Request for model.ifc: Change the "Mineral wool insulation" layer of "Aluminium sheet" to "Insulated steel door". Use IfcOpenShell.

First a look at what the model holds.

```python
import ifcopenshell
import ifcopenshell.util.element

model = ifcopenshell.open("model.ifc")
print(model.schema)
for layer_set in model.by_type("IfcMaterialLayerSet"):
    if layer_set.LayerSetName == "Aluminium sheet":
        for layer in layer_set.MaterialLayers:
            print(layer.id(), layer.Material and layer.Material.Name, layer.LayerThickness, sep=" | ")
        print(len(ifcopenshell.util.element.get_elements_by_material(model, layer_set)), "elements and types use it")
print(sorted(m.Name for m in model.by_type("IfcMaterial") if m.Name)[:60])
```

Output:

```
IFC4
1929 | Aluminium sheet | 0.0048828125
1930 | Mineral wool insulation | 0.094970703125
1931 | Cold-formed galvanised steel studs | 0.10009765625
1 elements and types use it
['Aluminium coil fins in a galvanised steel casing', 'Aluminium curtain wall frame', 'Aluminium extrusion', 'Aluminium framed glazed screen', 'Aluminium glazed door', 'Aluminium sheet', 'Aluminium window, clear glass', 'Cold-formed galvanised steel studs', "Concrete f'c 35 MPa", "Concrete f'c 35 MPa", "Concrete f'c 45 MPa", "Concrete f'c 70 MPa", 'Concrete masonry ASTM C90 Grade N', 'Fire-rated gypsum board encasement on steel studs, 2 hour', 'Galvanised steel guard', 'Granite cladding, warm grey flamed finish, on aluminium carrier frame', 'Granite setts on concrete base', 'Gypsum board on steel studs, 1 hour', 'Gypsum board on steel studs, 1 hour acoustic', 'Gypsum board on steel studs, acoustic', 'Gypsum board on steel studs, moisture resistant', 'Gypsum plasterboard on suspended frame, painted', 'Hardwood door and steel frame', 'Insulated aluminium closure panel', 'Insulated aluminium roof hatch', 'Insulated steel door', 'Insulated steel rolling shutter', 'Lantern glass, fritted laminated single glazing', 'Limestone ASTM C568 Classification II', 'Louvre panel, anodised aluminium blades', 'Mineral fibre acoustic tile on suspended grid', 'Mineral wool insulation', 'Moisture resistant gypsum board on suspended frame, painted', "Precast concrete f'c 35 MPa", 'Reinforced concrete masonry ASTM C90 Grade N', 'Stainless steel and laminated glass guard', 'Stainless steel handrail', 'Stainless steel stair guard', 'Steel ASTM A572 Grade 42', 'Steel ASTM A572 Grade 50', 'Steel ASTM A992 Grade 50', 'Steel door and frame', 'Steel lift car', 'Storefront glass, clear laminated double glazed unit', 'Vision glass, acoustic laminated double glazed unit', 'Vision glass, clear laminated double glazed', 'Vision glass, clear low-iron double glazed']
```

```python
import ifcopenshell
import ifcopenshell.api.material

model = ifcopenshell.open("model.ifc")

layer_set = next(s for s in model.by_type("IfcMaterialLayerSet") if s.LayerSetName == "Aluminium sheet")
layer = next(l for l in layer_set.MaterialLayers if l.Material and l.Material.Name == "Mineral wool insulation")
material = next(m for m in model.by_type("IfcMaterial") if m.Name == "Insulated steel door")

# Point this one layer at the other material; renaming the old one would change it everywhere.
ifcopenshell.api.material.edit_layer(model, layer=layer, attributes={}, material=material)

print([l.Material.Name if l.Material else None for l in layer_set.MaterialLayers])

model.write("model_rev.ifc")
```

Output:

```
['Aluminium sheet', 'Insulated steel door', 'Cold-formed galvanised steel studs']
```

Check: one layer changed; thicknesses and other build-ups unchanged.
